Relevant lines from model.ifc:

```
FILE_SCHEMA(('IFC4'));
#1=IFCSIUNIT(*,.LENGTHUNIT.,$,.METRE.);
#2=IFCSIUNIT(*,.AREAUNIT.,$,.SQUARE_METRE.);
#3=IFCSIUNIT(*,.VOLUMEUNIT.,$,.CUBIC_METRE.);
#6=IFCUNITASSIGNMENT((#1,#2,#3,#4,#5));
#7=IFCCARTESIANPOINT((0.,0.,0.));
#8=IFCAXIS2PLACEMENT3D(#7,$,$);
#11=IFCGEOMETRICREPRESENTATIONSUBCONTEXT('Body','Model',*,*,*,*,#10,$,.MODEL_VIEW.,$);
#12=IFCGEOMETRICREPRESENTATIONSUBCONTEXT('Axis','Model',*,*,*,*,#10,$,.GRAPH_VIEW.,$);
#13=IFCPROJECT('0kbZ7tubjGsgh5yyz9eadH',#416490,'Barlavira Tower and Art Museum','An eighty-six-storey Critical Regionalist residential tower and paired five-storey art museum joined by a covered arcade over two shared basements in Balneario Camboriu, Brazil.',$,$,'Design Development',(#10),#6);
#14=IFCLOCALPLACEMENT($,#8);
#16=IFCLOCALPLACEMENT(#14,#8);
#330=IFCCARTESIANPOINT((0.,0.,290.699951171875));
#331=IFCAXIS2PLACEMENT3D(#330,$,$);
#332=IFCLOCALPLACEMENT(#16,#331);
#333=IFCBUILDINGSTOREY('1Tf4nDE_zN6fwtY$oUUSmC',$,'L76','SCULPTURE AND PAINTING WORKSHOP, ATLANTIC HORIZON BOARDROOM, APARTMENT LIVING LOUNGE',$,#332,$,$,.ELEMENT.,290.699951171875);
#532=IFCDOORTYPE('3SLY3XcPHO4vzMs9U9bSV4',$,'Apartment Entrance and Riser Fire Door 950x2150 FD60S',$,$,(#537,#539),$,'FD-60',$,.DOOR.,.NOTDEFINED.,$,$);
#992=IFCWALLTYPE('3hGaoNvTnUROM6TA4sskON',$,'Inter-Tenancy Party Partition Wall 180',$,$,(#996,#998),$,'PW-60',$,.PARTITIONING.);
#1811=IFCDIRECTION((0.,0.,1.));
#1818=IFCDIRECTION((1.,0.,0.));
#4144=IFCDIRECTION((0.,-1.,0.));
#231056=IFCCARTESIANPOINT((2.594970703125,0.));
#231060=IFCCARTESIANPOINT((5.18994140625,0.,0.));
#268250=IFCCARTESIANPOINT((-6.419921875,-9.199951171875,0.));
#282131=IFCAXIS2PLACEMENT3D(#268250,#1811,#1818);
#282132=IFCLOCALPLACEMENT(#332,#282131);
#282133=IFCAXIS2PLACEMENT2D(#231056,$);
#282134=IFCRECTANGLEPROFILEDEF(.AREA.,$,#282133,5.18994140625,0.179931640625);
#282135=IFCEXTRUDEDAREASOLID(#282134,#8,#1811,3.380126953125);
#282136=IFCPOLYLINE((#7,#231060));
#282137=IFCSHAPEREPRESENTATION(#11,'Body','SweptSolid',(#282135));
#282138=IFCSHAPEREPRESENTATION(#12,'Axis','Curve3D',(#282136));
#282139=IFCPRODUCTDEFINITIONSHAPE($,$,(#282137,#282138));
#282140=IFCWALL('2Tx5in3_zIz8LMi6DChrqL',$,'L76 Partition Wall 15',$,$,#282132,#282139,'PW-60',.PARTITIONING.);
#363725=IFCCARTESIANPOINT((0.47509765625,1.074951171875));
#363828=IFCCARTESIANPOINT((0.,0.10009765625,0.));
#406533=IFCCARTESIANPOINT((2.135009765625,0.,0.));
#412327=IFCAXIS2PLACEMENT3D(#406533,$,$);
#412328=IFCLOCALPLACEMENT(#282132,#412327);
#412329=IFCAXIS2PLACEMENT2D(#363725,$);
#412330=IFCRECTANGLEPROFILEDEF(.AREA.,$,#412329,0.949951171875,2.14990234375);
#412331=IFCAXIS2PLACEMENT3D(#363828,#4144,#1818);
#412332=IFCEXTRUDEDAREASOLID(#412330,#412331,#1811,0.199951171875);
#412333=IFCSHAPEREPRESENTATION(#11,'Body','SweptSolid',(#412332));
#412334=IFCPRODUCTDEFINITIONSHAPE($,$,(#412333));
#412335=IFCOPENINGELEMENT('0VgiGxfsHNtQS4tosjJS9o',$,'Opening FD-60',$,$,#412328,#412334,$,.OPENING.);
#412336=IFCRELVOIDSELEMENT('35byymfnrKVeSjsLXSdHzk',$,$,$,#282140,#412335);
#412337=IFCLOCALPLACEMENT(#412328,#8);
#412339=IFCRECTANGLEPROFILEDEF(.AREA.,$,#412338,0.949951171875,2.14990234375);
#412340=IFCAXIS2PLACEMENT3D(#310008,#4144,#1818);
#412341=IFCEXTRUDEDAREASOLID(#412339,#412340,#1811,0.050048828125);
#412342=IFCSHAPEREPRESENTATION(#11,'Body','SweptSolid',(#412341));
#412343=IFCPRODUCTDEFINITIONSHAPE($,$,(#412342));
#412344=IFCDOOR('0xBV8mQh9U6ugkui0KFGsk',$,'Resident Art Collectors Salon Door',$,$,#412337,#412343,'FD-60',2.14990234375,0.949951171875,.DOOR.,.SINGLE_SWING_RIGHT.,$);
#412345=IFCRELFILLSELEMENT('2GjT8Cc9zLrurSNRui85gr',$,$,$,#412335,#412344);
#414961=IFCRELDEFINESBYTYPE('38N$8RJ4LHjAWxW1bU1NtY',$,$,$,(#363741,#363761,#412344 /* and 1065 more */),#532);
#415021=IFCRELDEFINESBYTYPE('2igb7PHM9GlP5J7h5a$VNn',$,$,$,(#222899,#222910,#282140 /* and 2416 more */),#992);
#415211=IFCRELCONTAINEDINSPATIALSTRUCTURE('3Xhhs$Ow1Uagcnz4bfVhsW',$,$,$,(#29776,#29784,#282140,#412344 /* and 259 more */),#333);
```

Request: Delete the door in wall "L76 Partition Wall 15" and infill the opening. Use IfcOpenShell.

```python
import ifcopenshell
import ifcopenshell.api.feature
import ifcopenshell.api.root
import ifcopenshell.geom
import ifcopenshell.util.shape

model = ifcopenshell.open("model.ifc")
settings = ifcopenshell.geom.settings()


def volume(element):
    """Net volume in cubic metres, openings subtracted."""
    shape = ifcopenshell.geom.create_shape(settings, element)
    return ifcopenshell.util.shape.get_volume(shape.geometry)


door = model.by_guid("0xBV8mQh9U6ugkui0KFGsk")
opening = door.FillsVoids[0].RelatingOpeningElement
wall = opening.VoidsElements[0].RelatingBuildingElement
before = volume(wall)

ifcopenshell.api.root.remove_product(model, product=door)
ifcopenshell.api.feature.remove_feature(model, feature=opening)

after = volume(wall)

print(f"wall volume {before:.3f} -> {after:.3f} m3")

model.write("model_edited.ifc")
```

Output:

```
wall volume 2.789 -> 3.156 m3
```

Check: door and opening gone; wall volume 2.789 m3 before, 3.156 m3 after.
